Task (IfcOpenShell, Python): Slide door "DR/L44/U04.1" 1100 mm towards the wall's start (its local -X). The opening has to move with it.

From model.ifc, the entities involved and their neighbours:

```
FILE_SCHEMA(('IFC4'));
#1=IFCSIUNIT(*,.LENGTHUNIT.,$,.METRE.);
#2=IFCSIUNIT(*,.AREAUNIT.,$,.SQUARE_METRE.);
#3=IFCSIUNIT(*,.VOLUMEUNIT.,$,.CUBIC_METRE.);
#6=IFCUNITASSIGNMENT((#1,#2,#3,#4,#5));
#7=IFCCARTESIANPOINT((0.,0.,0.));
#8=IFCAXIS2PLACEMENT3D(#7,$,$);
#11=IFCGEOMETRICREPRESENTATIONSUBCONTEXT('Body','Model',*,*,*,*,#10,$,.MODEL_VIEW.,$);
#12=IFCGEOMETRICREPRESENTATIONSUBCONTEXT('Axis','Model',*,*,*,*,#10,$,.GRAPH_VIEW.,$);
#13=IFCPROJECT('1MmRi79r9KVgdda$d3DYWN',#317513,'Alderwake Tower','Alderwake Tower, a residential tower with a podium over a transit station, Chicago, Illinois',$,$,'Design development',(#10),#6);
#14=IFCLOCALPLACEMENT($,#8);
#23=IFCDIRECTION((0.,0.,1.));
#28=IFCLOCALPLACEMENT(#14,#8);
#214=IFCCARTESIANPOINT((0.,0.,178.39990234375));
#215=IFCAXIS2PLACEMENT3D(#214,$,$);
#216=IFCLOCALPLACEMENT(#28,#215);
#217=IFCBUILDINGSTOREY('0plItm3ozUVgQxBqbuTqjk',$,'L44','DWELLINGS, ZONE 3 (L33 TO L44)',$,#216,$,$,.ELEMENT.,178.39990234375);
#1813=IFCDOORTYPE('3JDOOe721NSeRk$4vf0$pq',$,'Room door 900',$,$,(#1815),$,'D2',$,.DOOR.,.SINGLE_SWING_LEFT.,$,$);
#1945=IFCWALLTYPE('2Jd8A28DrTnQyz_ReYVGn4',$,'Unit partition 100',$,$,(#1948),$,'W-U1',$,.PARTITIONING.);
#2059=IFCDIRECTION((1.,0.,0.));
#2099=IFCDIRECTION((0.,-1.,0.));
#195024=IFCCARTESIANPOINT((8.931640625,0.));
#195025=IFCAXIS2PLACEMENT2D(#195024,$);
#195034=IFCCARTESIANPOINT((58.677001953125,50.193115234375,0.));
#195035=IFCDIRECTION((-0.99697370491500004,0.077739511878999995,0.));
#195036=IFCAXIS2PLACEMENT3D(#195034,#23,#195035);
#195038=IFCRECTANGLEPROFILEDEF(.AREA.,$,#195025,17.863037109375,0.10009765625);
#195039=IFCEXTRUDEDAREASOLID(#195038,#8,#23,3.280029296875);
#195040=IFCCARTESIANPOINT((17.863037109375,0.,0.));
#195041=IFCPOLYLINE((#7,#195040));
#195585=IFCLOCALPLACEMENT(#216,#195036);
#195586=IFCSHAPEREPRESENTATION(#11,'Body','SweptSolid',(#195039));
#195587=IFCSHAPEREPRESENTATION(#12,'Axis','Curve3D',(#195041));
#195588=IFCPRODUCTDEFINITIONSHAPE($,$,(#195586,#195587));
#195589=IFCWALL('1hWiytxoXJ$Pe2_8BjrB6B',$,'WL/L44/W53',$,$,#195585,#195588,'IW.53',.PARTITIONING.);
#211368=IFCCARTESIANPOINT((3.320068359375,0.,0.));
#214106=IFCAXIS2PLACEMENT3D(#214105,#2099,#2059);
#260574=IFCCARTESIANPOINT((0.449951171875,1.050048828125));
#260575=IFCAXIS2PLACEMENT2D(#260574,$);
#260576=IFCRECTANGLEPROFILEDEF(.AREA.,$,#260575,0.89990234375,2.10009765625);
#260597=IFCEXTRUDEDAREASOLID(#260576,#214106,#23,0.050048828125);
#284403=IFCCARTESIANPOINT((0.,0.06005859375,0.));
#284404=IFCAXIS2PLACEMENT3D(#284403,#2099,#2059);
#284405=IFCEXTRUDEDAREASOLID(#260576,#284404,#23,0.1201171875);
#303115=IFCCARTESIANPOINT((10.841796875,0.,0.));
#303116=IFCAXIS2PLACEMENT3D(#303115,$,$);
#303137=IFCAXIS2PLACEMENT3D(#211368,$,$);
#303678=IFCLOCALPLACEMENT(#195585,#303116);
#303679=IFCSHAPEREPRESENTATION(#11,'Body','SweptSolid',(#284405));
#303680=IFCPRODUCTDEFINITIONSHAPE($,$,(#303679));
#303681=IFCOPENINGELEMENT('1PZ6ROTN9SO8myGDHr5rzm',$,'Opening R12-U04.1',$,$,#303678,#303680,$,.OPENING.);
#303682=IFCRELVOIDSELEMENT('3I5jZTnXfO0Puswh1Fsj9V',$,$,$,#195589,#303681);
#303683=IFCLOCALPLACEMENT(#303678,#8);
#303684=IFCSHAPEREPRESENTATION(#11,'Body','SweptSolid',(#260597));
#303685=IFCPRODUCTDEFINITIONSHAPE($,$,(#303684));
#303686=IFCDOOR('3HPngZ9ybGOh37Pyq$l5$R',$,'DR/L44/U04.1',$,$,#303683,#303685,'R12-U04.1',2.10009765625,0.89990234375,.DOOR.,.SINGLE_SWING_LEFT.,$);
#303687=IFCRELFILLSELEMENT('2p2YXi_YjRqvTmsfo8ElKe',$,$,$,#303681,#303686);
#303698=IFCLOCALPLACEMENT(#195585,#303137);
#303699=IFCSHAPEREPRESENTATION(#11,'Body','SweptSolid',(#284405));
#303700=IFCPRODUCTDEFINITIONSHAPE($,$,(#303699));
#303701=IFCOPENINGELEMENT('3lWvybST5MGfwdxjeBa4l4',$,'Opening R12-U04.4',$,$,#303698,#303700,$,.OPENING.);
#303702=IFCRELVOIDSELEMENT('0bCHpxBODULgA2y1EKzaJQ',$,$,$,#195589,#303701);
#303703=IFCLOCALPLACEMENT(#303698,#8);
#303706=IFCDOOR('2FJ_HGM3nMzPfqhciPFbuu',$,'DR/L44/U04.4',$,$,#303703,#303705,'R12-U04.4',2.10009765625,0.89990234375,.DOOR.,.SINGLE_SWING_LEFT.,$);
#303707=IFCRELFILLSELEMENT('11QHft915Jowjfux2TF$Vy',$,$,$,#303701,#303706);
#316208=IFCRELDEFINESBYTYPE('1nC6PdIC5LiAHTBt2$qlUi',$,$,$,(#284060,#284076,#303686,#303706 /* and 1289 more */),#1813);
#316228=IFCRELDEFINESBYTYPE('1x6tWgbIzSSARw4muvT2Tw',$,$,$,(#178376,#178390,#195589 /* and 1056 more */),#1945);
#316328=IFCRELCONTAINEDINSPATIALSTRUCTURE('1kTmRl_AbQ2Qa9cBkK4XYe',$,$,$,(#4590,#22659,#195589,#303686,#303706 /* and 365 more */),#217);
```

```python
import ifcopenshell
import ifcopenshell.api.geometry
import ifcopenshell.util.placement
import ifcopenshell.util.unit

model = ifcopenshell.open("model.ifc")
unit_scale = ifcopenshell.util.unit.calculate_unit_scale(model)

door = model.by_guid("3HPngZ9ybGOh37Pyq$l5$R")
opening = door.FillsVoids[0].RelatingOpeningElement
wall = opening.VoidsElements[0].RelatingBuildingElement

wall_matrix = ifcopenshell.util.placement.get_local_placement(wall.ObjectPlacement)
shift = wall_matrix[:3, 0] * -1.1 / unit_scale
before = ifcopenshell.util.placement.get_local_placement(door.ObjectPlacement)[:3, 3].copy()

# The door is placed relative to its opening, so it follows when the opening moves.
matrix = ifcopenshell.util.placement.get_local_placement(opening.ObjectPlacement)
matrix[:3, 3] += shift
ifcopenshell.api.geometry.edit_object_placement(
    model, product=opening, matrix=matrix, is_si=False, should_transform_children=True
)

after = ifcopenshell.util.placement.get_local_placement(door.ObjectPlacement)[:3, 3]
print("door moved by", (after - before).round(3) + 0.0)

model.write("model_updated.ifc")
```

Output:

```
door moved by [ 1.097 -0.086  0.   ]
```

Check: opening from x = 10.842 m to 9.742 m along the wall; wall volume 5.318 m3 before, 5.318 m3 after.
